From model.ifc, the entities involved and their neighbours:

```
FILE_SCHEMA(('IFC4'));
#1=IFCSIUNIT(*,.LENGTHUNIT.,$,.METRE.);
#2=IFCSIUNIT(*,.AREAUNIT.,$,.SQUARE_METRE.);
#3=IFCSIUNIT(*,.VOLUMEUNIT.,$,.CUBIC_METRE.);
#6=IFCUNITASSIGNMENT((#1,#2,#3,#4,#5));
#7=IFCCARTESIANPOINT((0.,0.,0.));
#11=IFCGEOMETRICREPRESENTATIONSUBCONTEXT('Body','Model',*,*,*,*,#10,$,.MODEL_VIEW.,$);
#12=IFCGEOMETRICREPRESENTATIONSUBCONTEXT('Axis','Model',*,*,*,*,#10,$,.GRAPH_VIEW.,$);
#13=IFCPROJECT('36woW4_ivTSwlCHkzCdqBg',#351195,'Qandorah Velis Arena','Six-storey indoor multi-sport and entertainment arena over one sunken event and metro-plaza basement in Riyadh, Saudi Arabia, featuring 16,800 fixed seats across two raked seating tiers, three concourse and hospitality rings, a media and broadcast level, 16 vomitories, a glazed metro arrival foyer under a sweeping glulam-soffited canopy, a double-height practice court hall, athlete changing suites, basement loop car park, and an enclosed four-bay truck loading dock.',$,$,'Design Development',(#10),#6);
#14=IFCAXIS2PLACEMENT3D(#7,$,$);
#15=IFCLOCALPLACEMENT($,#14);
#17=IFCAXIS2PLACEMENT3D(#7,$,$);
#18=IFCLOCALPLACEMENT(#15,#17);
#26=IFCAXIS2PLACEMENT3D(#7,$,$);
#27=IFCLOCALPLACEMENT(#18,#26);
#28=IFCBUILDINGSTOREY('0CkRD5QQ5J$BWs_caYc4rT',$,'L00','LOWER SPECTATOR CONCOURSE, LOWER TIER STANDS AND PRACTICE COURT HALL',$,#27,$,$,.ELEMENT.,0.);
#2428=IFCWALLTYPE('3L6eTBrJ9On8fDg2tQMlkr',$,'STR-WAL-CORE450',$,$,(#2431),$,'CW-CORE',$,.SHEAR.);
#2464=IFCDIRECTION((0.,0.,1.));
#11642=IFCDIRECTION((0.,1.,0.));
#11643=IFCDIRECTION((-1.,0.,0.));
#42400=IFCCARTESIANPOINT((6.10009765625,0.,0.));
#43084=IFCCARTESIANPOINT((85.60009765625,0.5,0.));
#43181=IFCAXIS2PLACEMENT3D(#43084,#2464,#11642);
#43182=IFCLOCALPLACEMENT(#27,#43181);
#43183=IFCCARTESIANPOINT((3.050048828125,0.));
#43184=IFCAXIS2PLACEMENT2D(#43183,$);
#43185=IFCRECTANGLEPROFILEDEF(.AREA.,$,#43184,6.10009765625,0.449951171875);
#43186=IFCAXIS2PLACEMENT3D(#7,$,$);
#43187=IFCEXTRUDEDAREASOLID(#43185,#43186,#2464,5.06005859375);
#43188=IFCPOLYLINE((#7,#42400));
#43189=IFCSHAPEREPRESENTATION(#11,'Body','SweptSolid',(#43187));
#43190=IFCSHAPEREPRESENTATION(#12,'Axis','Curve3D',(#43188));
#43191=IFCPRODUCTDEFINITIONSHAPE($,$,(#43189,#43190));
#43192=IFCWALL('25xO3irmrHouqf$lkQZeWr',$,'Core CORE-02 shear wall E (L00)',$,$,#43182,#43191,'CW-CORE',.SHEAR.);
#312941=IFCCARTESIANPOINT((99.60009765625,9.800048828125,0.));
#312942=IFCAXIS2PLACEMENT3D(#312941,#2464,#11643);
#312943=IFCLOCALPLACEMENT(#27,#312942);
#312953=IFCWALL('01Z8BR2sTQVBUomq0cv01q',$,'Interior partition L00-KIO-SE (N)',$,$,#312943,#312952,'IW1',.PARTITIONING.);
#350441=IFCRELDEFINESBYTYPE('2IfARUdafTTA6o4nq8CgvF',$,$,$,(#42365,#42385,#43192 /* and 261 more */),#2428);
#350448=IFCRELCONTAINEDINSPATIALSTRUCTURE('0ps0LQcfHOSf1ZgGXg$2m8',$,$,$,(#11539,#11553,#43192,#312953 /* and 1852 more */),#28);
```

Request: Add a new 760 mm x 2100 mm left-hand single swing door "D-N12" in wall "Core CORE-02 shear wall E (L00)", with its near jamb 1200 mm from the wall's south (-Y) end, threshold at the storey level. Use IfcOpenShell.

```python
import numpy as np
import ifcopenshell
import ifcopenshell.api.feature
import ifcopenshell.api.geometry
import ifcopenshell.api.root
import ifcopenshell.api.spatial
import ifcopenshell.geom
import ifcopenshell.util.element
import ifcopenshell.util.placement
import ifcopenshell.util.representation
import ifcopenshell.util.shape
import ifcopenshell.util.unit

model = ifcopenshell.open("model.ifc")
unit_scale = ifcopenshell.util.unit.calculate_unit_scale(model)
settings = ifcopenshell.geom.settings()


def volume(element):
    """Net volume in cubic metres, openings subtracted."""
    shape = ifcopenshell.geom.create_shape(settings, element)
    return ifcopenshell.util.shape.get_volume(shape.geometry)


wall = model.by_guid("25xO3irmrHouqf$lkQZeWr")
storey = ifcopenshell.util.element.get_container(wall, ifc_class="IfcBuildingStorey")
context = ifcopenshell.util.representation.get_context(model, "Model", "Body", "MODEL_VIEW")
before = volume(wall)

width, height, from_end, sill = 0.76, 2.1, 1.2, 0.0  # metres

# The wall runs along its own X axis, and the end named is its -X end.
wall_shape = ifcopenshell.geom.create_shape(settings, wall)
x, y, z = ifcopenshell.util.shape.get_vertices(wall_shape.geometry).T
start = x.min() + from_end
face, thickness = float(y.min()), float(y.max() - y.min())
wall_matrix = ifcopenshell.util.placement.get_local_placement(wall.ObjectPlacement)
level = ifcopenshell.util.placement.get_local_placement(storey.ObjectPlacement)[2, 3]


def in_wall(x, y):
    """Placement at x, y metres in the wall's axes, at sill height."""
    matrix = wall_matrix.copy()
    matrix[:, 3] = wall_matrix @ np.array([x / unit_scale, y / unit_scale, 0.0, 1.0])
    matrix[2, 3] = level + sill / unit_scale
    return matrix


# Opening: a box that overshoots both wall faces by 50 mm.
opening = ifcopenshell.api.root.create_entity(model, ifc_class="IfcOpeningElement", predefined_type="OPENING")
box = ifcopenshell.api.geometry.add_wall_representation(
    model, context=context, length=width, height=height, thickness=thickness + 0.1
)
ifcopenshell.api.geometry.assign_representation(model, product=opening, representation=box)
ifcopenshell.api.geometry.edit_object_placement(model, product=opening, matrix=in_wall(start, face - 0.05), is_si=False)
ifcopenshell.api.feature.add_feature(model, feature=opening, element=wall)

door = ifcopenshell.api.root.create_entity(model, ifc_class="IfcDoor", name="D-N12", predefined_type="DOOR")
door.OverallWidth, door.OverallHeight = width / unit_scale, height / unit_scale
door.OperationType = "SINGLE_SWING_LEFT"
body = ifcopenshell.api.geometry.add_door_representation(
    model,
    context=context,
    overall_width=door.OverallWidth,
    overall_height=door.OverallHeight,
    operation_type="SINGLE_SWING_LEFT",
    lining_properties={"LiningDepth": thickness / unit_scale, "ThresholdDepth": thickness / unit_scale},
)
ifcopenshell.api.geometry.assign_representation(model, product=door, representation=body)
ifcopenshell.api.spatial.assign_container(model, products=[door], relating_structure=storey)
ifcopenshell.api.feature.add_filling(model, opening=opening, element=door)

# The lining spans the wall, so the door starts at the wall face.
ifcopenshell.api.geometry.edit_object_placement(model, product=door, matrix=in_wall(start, face), is_si=False)

after = volume(wall)

print(f"wall volume {before:.3f} -> {after:.3f} m3")

model.write("model-out.ifc")
```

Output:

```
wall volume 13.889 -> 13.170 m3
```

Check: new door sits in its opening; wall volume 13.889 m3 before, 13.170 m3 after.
